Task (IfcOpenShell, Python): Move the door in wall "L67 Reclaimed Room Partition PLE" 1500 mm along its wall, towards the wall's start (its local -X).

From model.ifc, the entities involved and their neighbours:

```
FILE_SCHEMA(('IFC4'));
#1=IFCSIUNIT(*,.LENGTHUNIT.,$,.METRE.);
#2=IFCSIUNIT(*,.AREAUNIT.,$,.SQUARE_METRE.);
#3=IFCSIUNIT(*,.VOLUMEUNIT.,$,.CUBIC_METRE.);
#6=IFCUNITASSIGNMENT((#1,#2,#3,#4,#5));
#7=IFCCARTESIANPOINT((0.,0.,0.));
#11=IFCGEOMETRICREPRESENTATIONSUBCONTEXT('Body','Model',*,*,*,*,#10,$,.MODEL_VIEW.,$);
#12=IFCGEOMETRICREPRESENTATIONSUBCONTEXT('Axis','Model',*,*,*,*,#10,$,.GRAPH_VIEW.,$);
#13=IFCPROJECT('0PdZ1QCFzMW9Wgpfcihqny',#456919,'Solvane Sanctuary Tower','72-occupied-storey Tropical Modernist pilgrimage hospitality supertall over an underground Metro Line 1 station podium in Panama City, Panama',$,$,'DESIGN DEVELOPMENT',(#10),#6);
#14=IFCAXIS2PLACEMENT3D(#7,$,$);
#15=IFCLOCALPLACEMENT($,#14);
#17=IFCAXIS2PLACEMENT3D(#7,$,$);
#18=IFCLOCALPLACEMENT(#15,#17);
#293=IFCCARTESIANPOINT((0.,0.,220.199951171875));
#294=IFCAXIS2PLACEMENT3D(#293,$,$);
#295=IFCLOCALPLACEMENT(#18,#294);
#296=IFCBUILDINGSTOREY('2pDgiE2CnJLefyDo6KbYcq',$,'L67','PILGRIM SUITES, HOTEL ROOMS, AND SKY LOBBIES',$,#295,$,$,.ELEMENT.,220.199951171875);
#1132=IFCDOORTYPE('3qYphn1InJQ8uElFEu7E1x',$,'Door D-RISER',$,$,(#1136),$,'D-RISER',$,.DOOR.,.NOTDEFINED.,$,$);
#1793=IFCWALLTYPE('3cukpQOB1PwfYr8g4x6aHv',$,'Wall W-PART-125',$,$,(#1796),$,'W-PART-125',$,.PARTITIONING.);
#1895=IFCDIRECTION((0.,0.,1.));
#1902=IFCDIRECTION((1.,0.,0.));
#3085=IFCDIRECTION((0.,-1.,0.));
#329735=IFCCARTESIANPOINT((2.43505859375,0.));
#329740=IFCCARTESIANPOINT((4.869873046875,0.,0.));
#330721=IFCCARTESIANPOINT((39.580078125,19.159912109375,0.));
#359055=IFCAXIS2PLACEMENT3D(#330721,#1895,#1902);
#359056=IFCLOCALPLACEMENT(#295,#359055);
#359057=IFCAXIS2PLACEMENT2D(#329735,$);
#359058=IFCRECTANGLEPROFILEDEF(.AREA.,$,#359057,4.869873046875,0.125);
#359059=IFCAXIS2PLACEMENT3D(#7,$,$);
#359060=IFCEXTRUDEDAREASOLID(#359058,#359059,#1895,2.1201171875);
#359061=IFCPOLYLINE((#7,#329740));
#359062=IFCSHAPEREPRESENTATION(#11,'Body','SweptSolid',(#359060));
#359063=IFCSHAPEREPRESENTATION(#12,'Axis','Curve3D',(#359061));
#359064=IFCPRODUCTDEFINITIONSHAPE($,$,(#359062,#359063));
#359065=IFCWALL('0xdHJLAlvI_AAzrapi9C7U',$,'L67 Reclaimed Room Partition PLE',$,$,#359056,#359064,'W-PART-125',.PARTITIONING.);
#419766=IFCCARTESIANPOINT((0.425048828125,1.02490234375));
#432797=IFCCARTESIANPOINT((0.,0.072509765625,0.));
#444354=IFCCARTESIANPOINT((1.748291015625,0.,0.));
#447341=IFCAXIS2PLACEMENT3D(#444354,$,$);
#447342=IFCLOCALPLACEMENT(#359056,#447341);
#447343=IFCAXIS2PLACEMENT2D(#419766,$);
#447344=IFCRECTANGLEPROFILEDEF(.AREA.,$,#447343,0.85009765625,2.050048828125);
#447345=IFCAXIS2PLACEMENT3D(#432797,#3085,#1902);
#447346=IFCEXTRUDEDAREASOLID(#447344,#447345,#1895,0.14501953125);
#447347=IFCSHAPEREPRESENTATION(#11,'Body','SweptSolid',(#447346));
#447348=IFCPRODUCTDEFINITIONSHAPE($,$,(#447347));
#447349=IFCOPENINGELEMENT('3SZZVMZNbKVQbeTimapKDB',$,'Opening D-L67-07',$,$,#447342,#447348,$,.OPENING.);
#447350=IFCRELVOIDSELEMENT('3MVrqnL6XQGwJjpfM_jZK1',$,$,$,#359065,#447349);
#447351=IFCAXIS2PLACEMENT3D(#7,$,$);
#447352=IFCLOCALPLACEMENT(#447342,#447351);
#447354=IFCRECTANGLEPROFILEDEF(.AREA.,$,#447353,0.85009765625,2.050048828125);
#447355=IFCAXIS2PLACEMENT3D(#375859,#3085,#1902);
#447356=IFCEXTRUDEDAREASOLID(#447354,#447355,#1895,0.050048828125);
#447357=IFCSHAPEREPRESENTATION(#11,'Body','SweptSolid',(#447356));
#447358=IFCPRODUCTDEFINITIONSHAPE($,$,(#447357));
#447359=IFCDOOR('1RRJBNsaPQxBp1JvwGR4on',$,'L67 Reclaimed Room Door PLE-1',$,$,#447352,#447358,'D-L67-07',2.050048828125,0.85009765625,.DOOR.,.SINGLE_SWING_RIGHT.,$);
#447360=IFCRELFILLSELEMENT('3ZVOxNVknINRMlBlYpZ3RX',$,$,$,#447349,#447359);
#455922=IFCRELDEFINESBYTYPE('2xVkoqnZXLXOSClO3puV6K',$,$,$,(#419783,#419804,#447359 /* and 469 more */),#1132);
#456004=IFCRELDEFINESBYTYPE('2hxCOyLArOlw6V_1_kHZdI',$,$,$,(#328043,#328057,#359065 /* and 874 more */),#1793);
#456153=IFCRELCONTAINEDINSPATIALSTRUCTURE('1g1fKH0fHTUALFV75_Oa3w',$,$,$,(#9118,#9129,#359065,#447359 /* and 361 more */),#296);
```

```python
import ifcopenshell
import ifcopenshell.api.geometry
import ifcopenshell.util.placement

model = ifcopenshell.open("model.ifc")

door = model.by_guid("1RRJBNsaPQxBp1JvwGR4on")
opening = door.FillsVoids[0].RelatingOpeningElement
wall = opening.VoidsElements[0].RelatingBuildingElement

wall_matrix = ifcopenshell.util.placement.get_local_placement(wall.ObjectPlacement)
shift = wall_matrix[:3, 0] * -1.5
before = ifcopenshell.util.placement.get_local_placement(door.ObjectPlacement)[:3, 3].copy()

# The door is placed relative to its opening, so it follows when the opening moves.
matrix = ifcopenshell.util.placement.get_local_placement(opening.ObjectPlacement)
matrix[:3, 3] += shift
ifcopenshell.api.geometry.edit_object_placement(
    model, product=opening, matrix=matrix, is_si=False, should_transform_children=True
)

after = ifcopenshell.util.placement.get_local_placement(door.ObjectPlacement)[:3, 3]
print("door moved by", (after - before).round(3) + 0.0)

model.write("model_v2.ifc")
```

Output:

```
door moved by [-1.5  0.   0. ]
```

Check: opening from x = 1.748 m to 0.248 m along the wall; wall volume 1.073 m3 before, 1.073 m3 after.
